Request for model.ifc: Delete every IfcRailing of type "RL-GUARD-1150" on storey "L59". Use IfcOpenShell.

First a look at what the model holds.

```python
import ifcopenshell
import ifcopenshell.util.element

model = ifcopenshell.open("model.ifc")
print(model.schema)
storey = next(s for s in model.by_type("IfcBuildingStorey") if s.Name == "L59")
railings = [e for e in ifcopenshell.util.element.get_decomposition(storey) if e.is_a("IfcRailing")]
seen = {}
for e in railings:
    element_type = ifcopenshell.util.element.get_type(e)
    name = element_type.Name if element_type not in (None, e) else None
    seen[name] = seen.get(name, 0) + 1
for name, count in sorted(seen.items(), key=str):
    print(count, "x", name)
```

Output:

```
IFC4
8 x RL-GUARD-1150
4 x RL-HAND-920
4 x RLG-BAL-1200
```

```python
import ifcopenshell
import ifcopenshell.api.root
import ifcopenshell.util.element

model = ifcopenshell.open("model.ifc")

storey = next(s for s in model.by_type("IfcBuildingStorey") if s.Name == "L59")
railings = [e for e in ifcopenshell.util.element.get_decomposition(storey) if e.is_a("IfcRailing")]
targets = [e for e in railings if (t := ifcopenshell.util.element.get_type(e)) not in (None, e) and t.Name == "RL-GUARD-1150"]

for e in targets:
    ifcopenshell.api.root.remove_product(model, product=e)
print(len(targets), "removed")

model.write("model_v2.ifc")
```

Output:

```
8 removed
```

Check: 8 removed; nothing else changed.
